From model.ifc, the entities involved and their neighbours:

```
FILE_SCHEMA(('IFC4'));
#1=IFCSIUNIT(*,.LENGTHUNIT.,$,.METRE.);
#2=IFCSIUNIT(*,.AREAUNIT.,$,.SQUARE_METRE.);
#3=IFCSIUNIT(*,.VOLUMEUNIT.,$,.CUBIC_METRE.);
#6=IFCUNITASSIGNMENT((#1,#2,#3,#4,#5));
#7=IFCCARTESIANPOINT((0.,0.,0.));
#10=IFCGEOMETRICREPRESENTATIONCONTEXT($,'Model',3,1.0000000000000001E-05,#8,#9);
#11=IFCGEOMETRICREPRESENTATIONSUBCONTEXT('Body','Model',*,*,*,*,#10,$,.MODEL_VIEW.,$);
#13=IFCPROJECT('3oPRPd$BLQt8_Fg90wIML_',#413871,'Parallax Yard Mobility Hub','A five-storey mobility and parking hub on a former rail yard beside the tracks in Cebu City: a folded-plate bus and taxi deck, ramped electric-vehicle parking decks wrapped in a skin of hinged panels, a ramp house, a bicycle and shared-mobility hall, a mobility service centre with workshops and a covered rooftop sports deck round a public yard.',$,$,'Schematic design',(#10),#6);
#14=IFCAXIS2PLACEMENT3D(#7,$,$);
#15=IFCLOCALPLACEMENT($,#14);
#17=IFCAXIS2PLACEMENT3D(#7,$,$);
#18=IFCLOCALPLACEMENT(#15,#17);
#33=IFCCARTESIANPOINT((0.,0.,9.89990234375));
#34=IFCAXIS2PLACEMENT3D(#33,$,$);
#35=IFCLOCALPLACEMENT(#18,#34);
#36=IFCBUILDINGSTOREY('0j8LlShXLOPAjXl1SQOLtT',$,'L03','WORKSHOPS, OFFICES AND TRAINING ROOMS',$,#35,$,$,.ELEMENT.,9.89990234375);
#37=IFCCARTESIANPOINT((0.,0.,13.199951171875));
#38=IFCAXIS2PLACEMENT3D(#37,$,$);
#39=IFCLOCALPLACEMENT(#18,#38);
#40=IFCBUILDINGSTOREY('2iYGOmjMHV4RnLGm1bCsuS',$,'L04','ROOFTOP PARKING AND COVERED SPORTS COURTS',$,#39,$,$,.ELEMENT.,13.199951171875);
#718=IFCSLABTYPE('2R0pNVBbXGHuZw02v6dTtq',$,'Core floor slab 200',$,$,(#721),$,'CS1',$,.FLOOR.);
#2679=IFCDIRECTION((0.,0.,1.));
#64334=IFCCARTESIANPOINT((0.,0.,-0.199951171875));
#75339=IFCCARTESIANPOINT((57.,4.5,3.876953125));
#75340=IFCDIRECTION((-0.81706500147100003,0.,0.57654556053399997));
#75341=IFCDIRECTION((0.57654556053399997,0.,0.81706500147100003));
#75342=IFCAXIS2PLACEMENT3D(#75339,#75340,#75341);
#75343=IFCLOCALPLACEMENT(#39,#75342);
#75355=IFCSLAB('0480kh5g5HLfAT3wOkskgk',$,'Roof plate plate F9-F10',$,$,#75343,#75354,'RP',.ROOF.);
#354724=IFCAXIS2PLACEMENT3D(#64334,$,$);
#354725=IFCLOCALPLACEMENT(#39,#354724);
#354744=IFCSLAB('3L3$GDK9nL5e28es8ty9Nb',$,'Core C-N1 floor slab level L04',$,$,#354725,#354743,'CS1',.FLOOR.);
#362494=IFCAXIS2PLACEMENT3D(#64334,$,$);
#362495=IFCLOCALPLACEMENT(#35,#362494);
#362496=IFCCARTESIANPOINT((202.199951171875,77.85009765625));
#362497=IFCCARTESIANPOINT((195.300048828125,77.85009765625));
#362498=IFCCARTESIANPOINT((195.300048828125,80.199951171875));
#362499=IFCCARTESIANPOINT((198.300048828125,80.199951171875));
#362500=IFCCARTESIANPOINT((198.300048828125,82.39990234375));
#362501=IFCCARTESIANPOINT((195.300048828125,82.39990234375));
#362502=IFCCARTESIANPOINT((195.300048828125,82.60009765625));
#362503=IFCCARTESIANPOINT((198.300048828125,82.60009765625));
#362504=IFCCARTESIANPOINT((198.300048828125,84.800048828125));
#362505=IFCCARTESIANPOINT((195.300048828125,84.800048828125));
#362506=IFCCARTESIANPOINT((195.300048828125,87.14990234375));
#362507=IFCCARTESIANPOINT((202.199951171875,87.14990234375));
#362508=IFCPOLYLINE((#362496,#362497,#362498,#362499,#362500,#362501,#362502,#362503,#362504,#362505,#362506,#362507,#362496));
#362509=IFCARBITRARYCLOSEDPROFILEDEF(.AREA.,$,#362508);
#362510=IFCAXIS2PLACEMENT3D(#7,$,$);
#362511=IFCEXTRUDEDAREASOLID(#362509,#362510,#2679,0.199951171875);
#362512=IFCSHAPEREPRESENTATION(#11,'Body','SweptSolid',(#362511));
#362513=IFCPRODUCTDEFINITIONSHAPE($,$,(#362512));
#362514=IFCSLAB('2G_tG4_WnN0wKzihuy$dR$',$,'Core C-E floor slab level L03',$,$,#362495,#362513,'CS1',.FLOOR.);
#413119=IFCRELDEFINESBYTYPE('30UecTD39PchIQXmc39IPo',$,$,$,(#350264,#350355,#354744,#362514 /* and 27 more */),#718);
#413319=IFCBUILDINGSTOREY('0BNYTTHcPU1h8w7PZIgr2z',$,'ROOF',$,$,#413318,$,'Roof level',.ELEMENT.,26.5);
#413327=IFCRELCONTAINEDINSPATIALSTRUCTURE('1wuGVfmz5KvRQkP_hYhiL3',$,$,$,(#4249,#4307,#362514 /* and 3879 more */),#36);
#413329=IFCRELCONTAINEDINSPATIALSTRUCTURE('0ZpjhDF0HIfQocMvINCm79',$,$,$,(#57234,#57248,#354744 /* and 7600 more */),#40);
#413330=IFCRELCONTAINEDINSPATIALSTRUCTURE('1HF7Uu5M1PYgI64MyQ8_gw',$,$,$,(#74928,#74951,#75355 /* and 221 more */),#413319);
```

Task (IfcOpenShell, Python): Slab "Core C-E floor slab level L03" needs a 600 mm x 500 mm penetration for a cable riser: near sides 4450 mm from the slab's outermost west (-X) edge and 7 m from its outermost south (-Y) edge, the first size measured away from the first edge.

```python
import numpy as np
import ifcopenshell
import ifcopenshell.api.feature
import ifcopenshell.api.geometry
import ifcopenshell.api.root
import ifcopenshell.geom
import ifcopenshell.util.placement
import ifcopenshell.util.representation
import ifcopenshell.util.shape
import ifcopenshell.util.unit

model = ifcopenshell.open("model.ifc")
unit_scale = ifcopenshell.util.unit.calculate_unit_scale(model)
settings = ifcopenshell.geom.settings()


def volume(element):
    """Net volume in cubic metres, openings subtracted."""
    shape = ifcopenshell.geom.create_shape(settings, element)
    return ifcopenshell.util.shape.get_volume(shape.geometry)


slab = model.by_guid("2G_tG4_WnN0wKzihuy$dR$")
before = volume(slab)

# Extent in the slab's own axes, in metres. The edges named are its -X and -Y sides.
slab_shape = ifcopenshell.geom.create_shape(settings, slab)
vertices = ifcopenshell.util.shape.get_vertices(slab_shape.geometry)
x_min, y_min, bottom = vertices.min(axis=0)
top = vertices[:, 2].max()

opening = ifcopenshell.api.root.create_entity(model, ifc_class="IfcOpeningElement", name="Cable riser opening", predefined_type="OPENING")
context = ifcopenshell.util.representation.get_context(model, "Model", "Body", "MODEL_VIEW")
width, depth = 0.6, 0.5
outline = [(0.0, 0.0), (width, 0.0), (width, depth), (0.0, depth), (0.0, 0.0)]
# Overshoot both faces by 50 mm so the cut is clean.
shape = ifcopenshell.api.geometry.add_slab_representation(
    model, context=context, depth=top - bottom + 0.1, polyline=outline
)
ifcopenshell.api.geometry.assign_representation(model, product=opening, representation=shape)

matrix = ifcopenshell.util.placement.get_local_placement(slab.ObjectPlacement)
matrix[:, 3] = matrix @ np.append(np.array([x_min + 4.45, y_min + 7, bottom - 0.05]) / unit_scale, 1.0)
ifcopenshell.api.geometry.edit_object_placement(model, product=opening, matrix=matrix, is_si=False)
ifcopenshell.api.feature.add_feature(model, feature=opening, element=slab)

after = volume(slab)

print(f"slab volume {before:.3f} -> {after:.3f} m3")

model.write("model_edited.ifc")
```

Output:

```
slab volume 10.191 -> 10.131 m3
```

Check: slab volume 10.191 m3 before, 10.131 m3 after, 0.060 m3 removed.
